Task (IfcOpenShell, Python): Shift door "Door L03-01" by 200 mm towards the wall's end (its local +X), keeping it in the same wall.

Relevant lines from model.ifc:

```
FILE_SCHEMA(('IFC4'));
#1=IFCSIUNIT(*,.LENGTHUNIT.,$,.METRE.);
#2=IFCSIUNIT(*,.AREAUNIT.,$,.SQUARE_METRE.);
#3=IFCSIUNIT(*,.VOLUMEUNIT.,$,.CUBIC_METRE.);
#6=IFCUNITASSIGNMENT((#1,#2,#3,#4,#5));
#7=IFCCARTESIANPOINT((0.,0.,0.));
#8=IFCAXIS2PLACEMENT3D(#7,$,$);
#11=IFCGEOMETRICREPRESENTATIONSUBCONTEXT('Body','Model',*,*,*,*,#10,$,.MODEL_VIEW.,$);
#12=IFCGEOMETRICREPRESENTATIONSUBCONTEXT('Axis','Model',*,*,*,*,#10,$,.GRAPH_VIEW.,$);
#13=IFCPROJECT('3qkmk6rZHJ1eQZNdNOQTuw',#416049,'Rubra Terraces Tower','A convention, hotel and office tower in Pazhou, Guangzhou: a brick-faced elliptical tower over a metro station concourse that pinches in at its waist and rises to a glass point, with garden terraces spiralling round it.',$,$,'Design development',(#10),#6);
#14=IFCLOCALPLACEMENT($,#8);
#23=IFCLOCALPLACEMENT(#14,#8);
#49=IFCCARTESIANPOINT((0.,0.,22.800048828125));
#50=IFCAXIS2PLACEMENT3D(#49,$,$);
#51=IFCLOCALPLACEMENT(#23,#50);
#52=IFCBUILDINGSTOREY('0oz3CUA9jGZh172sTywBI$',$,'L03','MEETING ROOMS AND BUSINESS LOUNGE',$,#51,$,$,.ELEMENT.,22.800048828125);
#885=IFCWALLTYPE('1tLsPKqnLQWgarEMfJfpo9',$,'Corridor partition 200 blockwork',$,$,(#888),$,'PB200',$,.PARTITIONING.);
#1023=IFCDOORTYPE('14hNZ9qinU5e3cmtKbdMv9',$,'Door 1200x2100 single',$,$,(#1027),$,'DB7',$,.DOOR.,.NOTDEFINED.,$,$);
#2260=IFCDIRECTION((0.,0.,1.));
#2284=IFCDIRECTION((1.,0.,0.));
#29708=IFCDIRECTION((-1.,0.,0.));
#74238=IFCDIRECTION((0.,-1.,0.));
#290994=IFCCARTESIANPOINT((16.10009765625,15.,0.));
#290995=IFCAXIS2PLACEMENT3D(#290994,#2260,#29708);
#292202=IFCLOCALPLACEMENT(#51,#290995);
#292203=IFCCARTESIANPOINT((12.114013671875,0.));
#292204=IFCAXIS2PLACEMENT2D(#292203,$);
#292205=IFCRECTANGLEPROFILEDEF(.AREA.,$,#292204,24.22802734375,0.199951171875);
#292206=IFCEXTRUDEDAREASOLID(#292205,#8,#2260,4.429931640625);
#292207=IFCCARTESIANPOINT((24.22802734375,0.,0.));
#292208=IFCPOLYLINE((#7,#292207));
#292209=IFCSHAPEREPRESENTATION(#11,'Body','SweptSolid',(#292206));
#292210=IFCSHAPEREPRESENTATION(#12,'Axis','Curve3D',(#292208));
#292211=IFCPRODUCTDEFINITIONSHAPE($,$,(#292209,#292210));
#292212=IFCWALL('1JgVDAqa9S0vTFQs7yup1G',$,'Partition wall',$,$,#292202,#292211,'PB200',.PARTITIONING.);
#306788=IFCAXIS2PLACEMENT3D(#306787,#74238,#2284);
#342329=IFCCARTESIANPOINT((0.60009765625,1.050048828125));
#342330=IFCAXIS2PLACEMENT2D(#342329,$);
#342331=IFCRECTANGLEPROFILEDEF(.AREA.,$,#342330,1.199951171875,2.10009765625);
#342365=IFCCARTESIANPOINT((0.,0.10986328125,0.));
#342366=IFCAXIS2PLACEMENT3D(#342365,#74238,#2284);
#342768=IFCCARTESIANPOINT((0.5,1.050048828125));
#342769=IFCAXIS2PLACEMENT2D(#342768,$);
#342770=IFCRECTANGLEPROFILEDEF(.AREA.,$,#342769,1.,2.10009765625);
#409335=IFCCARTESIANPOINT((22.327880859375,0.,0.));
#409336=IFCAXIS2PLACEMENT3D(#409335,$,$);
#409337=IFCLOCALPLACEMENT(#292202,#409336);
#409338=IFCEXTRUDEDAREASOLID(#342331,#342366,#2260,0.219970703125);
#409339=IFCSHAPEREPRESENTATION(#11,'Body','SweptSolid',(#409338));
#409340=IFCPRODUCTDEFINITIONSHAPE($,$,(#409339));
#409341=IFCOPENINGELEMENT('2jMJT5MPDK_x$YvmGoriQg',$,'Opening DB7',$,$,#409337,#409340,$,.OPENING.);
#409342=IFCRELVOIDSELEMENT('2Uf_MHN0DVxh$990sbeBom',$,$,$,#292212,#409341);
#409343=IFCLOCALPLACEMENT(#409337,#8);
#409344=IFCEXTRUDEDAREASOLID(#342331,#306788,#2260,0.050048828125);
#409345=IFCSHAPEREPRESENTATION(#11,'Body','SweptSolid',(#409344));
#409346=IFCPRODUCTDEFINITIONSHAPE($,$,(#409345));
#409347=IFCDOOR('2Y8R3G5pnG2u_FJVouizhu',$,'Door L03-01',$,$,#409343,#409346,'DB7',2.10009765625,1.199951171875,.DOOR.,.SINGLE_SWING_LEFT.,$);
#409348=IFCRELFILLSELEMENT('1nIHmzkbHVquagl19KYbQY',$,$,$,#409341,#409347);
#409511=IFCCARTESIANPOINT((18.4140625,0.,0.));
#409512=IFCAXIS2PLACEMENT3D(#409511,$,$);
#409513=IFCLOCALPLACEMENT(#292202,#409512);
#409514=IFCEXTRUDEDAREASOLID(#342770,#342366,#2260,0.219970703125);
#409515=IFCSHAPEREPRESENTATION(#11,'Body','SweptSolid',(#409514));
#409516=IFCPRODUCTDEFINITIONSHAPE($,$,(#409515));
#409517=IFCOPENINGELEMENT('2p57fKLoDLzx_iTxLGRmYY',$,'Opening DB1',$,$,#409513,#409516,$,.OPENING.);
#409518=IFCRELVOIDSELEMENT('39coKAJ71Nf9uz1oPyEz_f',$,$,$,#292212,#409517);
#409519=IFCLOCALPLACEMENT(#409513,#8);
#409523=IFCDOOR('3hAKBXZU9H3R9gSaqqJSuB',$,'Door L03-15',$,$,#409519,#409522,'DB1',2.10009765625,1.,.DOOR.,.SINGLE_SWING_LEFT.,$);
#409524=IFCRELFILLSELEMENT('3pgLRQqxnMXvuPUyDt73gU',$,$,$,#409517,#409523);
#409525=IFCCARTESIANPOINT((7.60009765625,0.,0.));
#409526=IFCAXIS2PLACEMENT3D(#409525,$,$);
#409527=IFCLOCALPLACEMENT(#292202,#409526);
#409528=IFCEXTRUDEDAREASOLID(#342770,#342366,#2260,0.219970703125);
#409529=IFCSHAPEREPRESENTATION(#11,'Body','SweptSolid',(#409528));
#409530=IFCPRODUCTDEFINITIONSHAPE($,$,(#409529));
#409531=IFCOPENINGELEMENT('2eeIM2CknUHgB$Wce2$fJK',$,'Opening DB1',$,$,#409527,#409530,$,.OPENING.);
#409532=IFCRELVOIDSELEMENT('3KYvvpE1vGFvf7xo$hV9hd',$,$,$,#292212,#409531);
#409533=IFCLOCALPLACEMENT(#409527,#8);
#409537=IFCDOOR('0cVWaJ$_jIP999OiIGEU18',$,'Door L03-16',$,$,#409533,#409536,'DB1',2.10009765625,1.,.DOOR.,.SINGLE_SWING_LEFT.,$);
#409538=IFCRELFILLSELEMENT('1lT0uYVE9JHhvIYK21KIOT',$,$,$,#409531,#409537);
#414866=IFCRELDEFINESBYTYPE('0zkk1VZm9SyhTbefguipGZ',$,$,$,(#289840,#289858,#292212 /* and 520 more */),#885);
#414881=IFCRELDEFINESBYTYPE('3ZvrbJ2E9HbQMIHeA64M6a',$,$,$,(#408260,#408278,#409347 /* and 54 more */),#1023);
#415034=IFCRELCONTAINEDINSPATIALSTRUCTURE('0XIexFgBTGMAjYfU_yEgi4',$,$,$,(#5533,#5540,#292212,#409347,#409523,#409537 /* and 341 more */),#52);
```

```python
import ifcopenshell
import ifcopenshell.api.geometry
import ifcopenshell.util.placement
import ifcopenshell.util.unit

model = ifcopenshell.open("model.ifc")
unit_scale = ifcopenshell.util.unit.calculate_unit_scale(model)

door = model.by_guid("2Y8R3G5pnG2u_FJVouizhu")
opening = door.FillsVoids[0].RelatingOpeningElement
wall = opening.VoidsElements[0].RelatingBuildingElement

wall_matrix = ifcopenshell.util.placement.get_local_placement(wall.ObjectPlacement)
shift = wall_matrix[:3, 0] * 0.2 / unit_scale
before = ifcopenshell.util.placement.get_local_placement(door.ObjectPlacement)[:3, 3].copy()

# The door is placed relative to its opening, so it follows when the opening moves.
matrix = ifcopenshell.util.placement.get_local_placement(opening.ObjectPlacement)
matrix[:3, 3] += shift
ifcopenshell.api.geometry.edit_object_placement(
    model, product=opening, matrix=matrix, is_si=False, should_transform_children=True
)

after = ifcopenshell.util.placement.get_local_placement(door.ObjectPlacement)[:3, 3]
print("door moved by", (after - before).round(3) + 0.0)

model.write("model-out.ifc")
```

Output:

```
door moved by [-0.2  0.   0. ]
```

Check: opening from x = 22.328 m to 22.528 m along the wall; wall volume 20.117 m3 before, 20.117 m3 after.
